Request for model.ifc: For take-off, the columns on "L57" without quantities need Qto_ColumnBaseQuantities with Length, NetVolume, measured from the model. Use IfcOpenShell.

First a look at what the model holds.

```python
import ifcopenshell
import ifcopenshell.util.element
import ifcopenshell.util.unit

model = ifcopenshell.open("model.ifc")
print(model.schema)
for unit_type in ("LENGTHUNIT", "AREAUNIT", "VOLUMEUNIT"):
    print(unit_type, ifcopenshell.util.unit.calculate_unit_scale(model, unit_type))
storey = next(s for s in model.by_type("IfcBuildingStorey") if s.Name == "L57")
columns = [e for e in ifcopenshell.util.element.get_decomposition(storey) if e.is_a("IfcColumn")]
for e in sorted(columns, key=lambda e: e.id()):
    print(e.id(), e.is_a(), e.Name, list(ifcopenshell.util.element.get_psets(e, qtos_only=True)), sep=" | ")
```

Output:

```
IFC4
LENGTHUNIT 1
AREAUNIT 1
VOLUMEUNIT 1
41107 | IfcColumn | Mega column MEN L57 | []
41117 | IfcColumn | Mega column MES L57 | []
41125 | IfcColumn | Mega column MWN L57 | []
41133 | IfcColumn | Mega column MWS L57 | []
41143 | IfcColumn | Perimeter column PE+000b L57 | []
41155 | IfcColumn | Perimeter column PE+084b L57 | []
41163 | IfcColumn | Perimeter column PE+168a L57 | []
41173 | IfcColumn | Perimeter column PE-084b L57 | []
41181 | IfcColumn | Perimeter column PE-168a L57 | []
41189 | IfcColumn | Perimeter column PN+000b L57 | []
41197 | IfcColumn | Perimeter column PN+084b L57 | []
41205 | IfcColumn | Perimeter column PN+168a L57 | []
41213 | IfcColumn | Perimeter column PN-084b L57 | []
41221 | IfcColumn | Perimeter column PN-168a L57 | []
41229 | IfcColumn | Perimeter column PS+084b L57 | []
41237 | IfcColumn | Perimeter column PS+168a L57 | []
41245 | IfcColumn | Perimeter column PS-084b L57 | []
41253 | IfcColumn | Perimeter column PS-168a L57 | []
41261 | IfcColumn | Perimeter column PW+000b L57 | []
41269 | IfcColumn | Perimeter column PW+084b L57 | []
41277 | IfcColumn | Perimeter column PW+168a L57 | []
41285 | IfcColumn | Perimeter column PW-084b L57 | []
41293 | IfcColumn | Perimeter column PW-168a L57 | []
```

```python
import ifcopenshell
import ifcopenshell.api.pset
import ifcopenshell.geom
import ifcopenshell.util.element
import ifcopenshell.util.shape
import ifcopenshell.util.unit

model = ifcopenshell.open("model.ifc")
unit_scale = ifcopenshell.util.unit.calculate_unit_scale(model)
volume_scale = ifcopenshell.util.unit.calculate_unit_scale(model, "VOLUMEUNIT")
settings = ifcopenshell.geom.settings()

storey = next(s for s in model.by_type("IfcBuildingStorey") if s.Name == "L57")
columns = [e for e in ifcopenshell.util.element.get_decomposition(storey) if e.is_a("IfcColumn")]

for e in sorted(columns, key=lambda e: e.id()):
    if ifcopenshell.util.element.get_psets(e, qtos_only=True, should_inherit=False):
        continue
    # Geometry comes back in metres, in the element's own axes.
    shape = ifcopenshell.geom.create_shape(settings, e)
    values = {
        "Length": ifcopenshell.util.shape.get_z(shape.geometry) / unit_scale,
        "NetVolume": ifcopenshell.util.shape.get_volume(shape.geometry) / volume_scale,
    }
    qto = ifcopenshell.api.pset.add_qto(model, product=e, name="Qto_ColumnBaseQuantities")
    ifcopenshell.api.pset.edit_qto(model, qto=qto, properties=values)
    print(e.id(), {k: round(v, 3) for k, v in values.items()})

model.write("model_v2.ifc")
```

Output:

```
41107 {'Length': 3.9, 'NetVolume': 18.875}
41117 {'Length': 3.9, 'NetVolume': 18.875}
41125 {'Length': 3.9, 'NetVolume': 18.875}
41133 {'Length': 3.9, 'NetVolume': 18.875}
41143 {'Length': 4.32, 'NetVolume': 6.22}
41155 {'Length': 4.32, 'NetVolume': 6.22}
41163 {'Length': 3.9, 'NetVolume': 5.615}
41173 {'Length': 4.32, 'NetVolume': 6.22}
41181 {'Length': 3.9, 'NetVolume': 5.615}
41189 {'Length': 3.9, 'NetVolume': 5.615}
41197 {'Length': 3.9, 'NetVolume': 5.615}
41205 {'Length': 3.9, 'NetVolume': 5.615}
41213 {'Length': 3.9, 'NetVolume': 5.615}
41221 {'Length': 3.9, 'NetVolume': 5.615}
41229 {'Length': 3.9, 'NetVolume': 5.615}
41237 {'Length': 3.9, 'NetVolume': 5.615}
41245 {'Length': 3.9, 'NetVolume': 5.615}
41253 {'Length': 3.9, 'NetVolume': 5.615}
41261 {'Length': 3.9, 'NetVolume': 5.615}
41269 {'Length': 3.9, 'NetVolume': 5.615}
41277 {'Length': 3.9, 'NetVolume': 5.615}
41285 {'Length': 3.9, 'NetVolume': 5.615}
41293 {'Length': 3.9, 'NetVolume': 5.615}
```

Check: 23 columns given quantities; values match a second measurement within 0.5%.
